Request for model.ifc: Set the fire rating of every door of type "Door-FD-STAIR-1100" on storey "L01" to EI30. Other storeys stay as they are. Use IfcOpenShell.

First a look at what the model holds.

```python
import ifcopenshell
import ifcopenshell.util.element

model = ifcopenshell.open("model.ifc")
print(model.schema)
storey = next(s for s in model.by_type("IfcBuildingStorey") if s.Name == "L01")
doors = [e for e in ifcopenshell.util.element.get_decomposition(storey) if e.is_a("IfcDoor")]
seen = {}
for e in doors:
    element_type = ifcopenshell.util.element.get_type(e)
    key = (element_type.Name if element_type != e and element_type else None, ifcopenshell.util.element.get_pset(e, "Pset_DoorCommon", "FireRating"))
    seen[key] = seen.get(key, 0) + 1
for (name, value), count in sorted(seen.items(), key=str):
    print(count, "x", name, "|", value)
```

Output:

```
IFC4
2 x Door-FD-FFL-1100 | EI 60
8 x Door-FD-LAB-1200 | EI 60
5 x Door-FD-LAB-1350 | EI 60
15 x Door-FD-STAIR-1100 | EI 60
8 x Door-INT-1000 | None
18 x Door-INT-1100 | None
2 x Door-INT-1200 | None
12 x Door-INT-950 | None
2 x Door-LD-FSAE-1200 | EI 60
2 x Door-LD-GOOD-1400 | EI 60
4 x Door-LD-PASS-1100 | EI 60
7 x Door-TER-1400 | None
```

```python
import ifcopenshell
import ifcopenshell.api.pset
import ifcopenshell.util.element

model = ifcopenshell.open("model.ifc")

storey = next(s for s in model.by_type("IfcBuildingStorey") if s.Name == "L01")
doors = [e for e in ifcopenshell.util.element.get_decomposition(storey) if e.is_a("IfcDoor")]

count = 0
for e in doors:
    element_type = ifcopenshell.util.element.get_type(e)
    if element_type in (None, e) or element_type.Name != "Door-FD-STAIR-1100":
        continue
    # add_pset returns the element's existing set when there is one.
    pset = ifcopenshell.api.pset.add_pset(model, product=e, name="Pset_DoorCommon")
    ifcopenshell.api.pset.edit_pset(model, pset=pset, properties={"FireRating": "EI30"})
    count += 1

print(count, "doors updated")

model.write("model_rev.ifc")
```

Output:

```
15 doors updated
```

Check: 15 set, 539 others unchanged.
